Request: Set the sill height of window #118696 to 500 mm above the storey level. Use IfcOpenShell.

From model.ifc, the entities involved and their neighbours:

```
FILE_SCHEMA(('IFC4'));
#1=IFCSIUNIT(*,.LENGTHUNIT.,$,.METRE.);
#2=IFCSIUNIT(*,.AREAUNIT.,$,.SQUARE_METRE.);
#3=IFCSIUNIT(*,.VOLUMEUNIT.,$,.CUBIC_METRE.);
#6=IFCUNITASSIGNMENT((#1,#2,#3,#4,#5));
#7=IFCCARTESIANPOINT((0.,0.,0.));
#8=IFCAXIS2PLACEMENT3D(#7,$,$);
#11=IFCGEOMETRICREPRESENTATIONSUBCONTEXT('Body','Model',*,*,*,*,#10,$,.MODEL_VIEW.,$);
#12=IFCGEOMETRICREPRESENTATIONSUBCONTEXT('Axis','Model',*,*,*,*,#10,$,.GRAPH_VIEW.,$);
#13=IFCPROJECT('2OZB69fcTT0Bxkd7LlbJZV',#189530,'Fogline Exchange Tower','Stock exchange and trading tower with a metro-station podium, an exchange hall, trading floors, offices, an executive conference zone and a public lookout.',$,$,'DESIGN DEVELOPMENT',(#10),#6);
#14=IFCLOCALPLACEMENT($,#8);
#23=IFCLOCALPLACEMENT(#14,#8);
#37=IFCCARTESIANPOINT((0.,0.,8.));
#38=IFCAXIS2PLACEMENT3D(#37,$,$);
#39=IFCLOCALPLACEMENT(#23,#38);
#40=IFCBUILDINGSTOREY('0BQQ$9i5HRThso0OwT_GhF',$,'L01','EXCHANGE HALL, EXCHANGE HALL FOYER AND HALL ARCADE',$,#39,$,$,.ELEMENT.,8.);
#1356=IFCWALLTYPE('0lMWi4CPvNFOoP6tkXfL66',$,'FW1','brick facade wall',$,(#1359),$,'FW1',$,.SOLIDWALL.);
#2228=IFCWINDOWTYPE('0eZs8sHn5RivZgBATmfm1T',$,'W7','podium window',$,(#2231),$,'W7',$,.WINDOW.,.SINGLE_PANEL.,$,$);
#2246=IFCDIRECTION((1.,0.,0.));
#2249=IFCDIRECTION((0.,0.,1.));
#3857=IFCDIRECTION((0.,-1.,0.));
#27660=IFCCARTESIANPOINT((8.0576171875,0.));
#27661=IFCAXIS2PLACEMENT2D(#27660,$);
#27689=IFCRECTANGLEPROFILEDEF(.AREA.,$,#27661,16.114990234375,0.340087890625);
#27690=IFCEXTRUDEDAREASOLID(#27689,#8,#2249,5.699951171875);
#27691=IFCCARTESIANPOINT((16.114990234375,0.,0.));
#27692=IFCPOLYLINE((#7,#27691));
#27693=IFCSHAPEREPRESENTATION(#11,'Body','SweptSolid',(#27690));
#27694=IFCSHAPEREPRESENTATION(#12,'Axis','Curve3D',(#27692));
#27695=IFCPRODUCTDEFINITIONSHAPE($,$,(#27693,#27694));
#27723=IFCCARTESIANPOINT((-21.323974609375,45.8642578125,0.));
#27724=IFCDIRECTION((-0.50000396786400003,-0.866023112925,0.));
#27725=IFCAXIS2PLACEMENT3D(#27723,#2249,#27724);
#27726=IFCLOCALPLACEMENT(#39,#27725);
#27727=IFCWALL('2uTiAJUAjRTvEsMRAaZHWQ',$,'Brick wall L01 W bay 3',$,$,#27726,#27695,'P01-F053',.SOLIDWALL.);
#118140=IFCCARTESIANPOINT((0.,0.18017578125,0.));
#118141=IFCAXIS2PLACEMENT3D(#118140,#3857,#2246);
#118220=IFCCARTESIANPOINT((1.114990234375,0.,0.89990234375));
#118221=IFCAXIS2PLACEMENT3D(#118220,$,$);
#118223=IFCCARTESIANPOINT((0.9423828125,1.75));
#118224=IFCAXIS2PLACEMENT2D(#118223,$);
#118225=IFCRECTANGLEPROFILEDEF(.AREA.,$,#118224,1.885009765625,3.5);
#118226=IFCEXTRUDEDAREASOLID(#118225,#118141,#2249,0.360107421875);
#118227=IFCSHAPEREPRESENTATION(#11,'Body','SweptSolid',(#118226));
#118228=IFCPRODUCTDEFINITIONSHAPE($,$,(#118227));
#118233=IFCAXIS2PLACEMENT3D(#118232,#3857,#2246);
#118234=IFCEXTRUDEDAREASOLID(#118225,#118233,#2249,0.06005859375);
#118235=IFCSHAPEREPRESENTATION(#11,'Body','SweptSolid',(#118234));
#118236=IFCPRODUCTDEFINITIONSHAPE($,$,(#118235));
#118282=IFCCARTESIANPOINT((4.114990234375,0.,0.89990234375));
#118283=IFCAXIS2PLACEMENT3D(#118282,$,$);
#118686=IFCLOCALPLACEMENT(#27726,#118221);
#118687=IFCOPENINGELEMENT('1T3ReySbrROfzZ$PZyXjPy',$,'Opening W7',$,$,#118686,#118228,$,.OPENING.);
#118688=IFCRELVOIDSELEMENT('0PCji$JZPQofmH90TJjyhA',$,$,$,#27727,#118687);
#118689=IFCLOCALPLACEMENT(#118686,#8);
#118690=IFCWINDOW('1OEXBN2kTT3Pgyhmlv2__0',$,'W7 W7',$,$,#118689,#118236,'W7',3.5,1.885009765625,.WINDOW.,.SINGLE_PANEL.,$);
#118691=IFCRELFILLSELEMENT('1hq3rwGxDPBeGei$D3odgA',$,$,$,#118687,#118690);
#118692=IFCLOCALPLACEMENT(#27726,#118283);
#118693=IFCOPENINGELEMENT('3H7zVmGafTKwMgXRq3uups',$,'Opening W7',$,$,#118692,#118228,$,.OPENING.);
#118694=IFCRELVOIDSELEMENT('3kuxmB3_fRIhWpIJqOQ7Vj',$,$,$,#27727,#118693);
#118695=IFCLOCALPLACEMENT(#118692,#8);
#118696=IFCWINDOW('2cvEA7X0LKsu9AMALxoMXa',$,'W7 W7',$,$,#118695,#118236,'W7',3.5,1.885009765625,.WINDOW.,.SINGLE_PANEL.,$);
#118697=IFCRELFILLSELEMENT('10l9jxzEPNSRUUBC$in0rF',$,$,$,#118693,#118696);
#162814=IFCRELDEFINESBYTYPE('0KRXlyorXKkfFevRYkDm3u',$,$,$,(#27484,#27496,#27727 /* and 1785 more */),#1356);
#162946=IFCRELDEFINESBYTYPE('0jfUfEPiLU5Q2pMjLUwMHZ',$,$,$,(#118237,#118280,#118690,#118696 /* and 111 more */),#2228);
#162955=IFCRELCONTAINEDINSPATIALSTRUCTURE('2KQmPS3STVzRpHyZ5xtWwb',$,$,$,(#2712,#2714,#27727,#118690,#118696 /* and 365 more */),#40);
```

```python
import numpy as np
import ifcopenshell
import ifcopenshell.api.geometry
import ifcopenshell.geom
import ifcopenshell.util.element
import ifcopenshell.util.placement
import ifcopenshell.util.shape
import ifcopenshell.util.unit

model = ifcopenshell.open("model.ifc")
unit_scale = ifcopenshell.util.unit.calculate_unit_scale(model)

window = model.by_guid("2cvEA7X0LKsu9AMALxoMXa")
opening = window.FillsVoids[0].RelatingOpeningElement
storey = ifcopenshell.util.element.get_container(window, ifc_class="IfcBuildingStorey")
level = ifcopenshell.util.placement.get_local_placement(storey.ObjectPlacement)[2, 3]

# The opening's origin need not be at the sill, so measure its lowest point.
shape = ifcopenshell.geom.create_shape(ifcopenshell.geom.settings(), opening)
bottom = ifcopenshell.util.shape.get_shape_bottom_elevation(shape, shape.geometry) / unit_scale
dz = level + 0.5 - bottom

shift = np.array([0.0, 0.0, dz])
# The window is placed relative to its opening, so it follows when the opening moves.
matrix = ifcopenshell.util.placement.get_local_placement(opening.ObjectPlacement)
matrix[:3, 3] += shift
ifcopenshell.api.geometry.edit_object_placement(
    model, product=opening, matrix=matrix, is_si=False, should_transform_children=True
)

print(f"moved by {dz * unit_scale:+.3f} m")

model.write("model_updated.ifc")
```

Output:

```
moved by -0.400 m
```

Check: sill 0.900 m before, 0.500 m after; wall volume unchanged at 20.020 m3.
